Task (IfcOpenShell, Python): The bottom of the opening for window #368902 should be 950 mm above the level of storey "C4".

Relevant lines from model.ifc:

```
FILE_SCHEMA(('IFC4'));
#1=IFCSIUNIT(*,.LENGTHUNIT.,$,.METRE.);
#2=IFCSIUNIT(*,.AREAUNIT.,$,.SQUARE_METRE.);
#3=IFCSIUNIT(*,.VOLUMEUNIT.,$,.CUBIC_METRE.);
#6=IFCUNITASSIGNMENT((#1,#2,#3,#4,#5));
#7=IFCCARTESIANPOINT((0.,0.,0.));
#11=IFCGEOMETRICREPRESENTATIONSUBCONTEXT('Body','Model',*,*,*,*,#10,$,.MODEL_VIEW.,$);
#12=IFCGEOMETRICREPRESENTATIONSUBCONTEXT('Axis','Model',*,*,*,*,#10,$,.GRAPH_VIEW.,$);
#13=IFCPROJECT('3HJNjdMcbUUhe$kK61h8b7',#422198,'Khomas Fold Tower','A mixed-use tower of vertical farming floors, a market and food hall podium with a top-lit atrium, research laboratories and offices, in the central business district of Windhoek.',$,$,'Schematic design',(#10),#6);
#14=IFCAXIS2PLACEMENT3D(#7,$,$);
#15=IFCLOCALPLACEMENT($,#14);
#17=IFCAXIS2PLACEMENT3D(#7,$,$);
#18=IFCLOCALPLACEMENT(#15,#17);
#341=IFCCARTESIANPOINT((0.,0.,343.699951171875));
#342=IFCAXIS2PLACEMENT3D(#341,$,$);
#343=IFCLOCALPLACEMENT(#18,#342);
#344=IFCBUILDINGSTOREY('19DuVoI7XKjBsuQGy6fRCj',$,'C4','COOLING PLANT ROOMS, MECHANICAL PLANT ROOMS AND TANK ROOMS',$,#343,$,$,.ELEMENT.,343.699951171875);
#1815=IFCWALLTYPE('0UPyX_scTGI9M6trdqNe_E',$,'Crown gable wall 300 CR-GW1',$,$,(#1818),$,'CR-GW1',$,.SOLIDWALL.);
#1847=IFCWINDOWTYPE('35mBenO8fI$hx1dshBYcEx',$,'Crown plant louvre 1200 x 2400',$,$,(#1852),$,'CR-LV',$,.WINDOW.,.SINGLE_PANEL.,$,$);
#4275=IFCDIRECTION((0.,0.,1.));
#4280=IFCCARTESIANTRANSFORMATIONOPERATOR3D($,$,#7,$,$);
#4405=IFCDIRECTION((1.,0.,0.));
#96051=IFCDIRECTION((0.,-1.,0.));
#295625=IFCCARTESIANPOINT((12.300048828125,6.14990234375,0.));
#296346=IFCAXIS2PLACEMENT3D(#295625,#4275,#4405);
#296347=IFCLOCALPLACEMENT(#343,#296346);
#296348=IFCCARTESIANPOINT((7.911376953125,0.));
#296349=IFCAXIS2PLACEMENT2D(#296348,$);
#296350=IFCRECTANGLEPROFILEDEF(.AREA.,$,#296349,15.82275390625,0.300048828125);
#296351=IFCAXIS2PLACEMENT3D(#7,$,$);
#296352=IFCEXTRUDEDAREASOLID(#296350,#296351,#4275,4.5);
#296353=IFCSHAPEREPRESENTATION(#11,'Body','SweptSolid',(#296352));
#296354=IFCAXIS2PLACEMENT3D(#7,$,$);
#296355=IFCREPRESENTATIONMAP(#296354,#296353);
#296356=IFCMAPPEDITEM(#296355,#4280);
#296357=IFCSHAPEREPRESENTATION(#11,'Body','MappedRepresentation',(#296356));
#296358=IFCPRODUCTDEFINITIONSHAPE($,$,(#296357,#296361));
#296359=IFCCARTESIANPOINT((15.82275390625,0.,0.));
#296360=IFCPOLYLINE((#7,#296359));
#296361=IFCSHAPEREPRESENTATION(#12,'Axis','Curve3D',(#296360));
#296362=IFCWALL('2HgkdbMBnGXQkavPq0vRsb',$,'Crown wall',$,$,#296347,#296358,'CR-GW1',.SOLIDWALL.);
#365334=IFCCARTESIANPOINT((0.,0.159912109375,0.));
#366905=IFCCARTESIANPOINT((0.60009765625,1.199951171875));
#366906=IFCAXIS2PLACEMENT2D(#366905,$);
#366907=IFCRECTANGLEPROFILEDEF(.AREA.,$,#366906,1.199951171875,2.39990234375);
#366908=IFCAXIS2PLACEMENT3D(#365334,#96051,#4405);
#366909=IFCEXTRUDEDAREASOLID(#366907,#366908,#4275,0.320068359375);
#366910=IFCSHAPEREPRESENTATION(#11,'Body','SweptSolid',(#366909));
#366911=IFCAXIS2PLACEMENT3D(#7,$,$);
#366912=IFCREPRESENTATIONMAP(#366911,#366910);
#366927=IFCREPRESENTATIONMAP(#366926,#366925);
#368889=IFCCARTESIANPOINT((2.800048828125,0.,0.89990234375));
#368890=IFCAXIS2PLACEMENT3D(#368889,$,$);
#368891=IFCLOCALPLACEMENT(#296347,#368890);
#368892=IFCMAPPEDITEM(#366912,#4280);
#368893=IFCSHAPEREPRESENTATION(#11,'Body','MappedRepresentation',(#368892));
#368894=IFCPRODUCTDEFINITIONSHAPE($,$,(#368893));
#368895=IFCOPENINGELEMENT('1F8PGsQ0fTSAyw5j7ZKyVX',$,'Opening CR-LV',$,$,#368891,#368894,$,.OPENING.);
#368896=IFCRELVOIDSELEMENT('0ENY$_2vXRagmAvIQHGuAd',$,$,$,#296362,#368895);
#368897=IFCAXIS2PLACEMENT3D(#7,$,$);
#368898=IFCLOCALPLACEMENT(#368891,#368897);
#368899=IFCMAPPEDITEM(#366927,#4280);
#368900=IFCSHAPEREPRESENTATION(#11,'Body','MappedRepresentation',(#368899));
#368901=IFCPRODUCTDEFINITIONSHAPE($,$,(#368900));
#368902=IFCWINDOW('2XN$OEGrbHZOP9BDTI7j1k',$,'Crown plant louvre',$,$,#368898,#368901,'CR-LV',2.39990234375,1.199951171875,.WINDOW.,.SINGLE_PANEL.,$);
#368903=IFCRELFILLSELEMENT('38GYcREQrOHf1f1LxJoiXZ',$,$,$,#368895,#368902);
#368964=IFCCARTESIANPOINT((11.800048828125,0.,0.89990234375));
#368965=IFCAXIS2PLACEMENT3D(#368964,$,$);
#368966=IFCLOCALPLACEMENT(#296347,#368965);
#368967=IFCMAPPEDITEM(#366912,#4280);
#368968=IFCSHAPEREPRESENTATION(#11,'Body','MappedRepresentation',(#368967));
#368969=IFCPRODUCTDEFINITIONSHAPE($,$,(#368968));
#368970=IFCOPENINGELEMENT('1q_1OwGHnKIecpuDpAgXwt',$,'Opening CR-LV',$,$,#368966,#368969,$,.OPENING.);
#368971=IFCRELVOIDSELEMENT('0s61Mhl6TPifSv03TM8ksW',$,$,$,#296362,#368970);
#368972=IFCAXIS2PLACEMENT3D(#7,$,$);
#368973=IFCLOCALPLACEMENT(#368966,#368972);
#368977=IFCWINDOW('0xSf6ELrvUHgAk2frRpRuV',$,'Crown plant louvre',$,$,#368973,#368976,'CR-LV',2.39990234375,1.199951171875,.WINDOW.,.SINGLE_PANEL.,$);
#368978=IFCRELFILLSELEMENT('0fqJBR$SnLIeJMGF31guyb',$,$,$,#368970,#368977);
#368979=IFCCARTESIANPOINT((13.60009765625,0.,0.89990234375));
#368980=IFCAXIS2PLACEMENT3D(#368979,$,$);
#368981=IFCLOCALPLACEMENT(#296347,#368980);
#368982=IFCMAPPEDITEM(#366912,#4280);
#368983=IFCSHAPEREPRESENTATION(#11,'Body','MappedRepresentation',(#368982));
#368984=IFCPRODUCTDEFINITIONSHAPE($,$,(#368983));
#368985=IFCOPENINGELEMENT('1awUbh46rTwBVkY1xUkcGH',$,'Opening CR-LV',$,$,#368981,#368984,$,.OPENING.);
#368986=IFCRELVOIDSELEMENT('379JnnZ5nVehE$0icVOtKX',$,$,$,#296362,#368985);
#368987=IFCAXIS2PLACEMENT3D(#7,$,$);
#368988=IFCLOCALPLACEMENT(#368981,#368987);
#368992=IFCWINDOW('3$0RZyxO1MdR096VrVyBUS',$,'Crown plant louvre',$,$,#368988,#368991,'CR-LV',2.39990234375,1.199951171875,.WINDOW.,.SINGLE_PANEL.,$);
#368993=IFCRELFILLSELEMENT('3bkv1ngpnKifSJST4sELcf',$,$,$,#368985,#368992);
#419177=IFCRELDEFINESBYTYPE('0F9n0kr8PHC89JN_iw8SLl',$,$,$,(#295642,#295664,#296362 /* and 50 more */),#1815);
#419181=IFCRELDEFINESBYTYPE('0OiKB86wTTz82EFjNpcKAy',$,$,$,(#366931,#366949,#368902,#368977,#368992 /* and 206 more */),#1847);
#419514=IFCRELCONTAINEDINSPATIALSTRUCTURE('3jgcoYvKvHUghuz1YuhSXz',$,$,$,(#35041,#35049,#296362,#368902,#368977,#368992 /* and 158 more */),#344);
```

```python
import numpy as np
import ifcopenshell
import ifcopenshell.api.geometry
import ifcopenshell.geom
import ifcopenshell.util.element
import ifcopenshell.util.placement
import ifcopenshell.util.shape
import ifcopenshell.util.unit

model = ifcopenshell.open("model.ifc")
unit_scale = ifcopenshell.util.unit.calculate_unit_scale(model)

window = model.by_id(368902)
opening = window.FillsVoids[0].RelatingOpeningElement
storey = ifcopenshell.util.element.get_container(window, ifc_class="IfcBuildingStorey")
level = ifcopenshell.util.placement.get_local_placement(storey.ObjectPlacement)[2, 3]

# The opening's origin need not be at the sill, so measure its lowest point.
shape = ifcopenshell.geom.create_shape(ifcopenshell.geom.settings(), opening)
bottom = ifcopenshell.util.shape.get_shape_bottom_elevation(shape, shape.geometry) / unit_scale
dz = level + 0.95 - bottom

shift = np.array([0.0, 0.0, dz])
# The window is placed relative to its opening, so it follows when the opening moves.
matrix = ifcopenshell.util.placement.get_local_placement(opening.ObjectPlacement)
matrix[:3, 3] += shift
ifcopenshell.api.geometry.edit_object_placement(
    model, product=opening, matrix=matrix, is_si=False, should_transform_children=True
)

print(f"moved by {dz * unit_scale:+.3f} m")

model.write("model_v2.ifc")
```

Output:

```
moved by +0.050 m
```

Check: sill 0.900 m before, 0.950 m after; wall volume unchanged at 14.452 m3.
